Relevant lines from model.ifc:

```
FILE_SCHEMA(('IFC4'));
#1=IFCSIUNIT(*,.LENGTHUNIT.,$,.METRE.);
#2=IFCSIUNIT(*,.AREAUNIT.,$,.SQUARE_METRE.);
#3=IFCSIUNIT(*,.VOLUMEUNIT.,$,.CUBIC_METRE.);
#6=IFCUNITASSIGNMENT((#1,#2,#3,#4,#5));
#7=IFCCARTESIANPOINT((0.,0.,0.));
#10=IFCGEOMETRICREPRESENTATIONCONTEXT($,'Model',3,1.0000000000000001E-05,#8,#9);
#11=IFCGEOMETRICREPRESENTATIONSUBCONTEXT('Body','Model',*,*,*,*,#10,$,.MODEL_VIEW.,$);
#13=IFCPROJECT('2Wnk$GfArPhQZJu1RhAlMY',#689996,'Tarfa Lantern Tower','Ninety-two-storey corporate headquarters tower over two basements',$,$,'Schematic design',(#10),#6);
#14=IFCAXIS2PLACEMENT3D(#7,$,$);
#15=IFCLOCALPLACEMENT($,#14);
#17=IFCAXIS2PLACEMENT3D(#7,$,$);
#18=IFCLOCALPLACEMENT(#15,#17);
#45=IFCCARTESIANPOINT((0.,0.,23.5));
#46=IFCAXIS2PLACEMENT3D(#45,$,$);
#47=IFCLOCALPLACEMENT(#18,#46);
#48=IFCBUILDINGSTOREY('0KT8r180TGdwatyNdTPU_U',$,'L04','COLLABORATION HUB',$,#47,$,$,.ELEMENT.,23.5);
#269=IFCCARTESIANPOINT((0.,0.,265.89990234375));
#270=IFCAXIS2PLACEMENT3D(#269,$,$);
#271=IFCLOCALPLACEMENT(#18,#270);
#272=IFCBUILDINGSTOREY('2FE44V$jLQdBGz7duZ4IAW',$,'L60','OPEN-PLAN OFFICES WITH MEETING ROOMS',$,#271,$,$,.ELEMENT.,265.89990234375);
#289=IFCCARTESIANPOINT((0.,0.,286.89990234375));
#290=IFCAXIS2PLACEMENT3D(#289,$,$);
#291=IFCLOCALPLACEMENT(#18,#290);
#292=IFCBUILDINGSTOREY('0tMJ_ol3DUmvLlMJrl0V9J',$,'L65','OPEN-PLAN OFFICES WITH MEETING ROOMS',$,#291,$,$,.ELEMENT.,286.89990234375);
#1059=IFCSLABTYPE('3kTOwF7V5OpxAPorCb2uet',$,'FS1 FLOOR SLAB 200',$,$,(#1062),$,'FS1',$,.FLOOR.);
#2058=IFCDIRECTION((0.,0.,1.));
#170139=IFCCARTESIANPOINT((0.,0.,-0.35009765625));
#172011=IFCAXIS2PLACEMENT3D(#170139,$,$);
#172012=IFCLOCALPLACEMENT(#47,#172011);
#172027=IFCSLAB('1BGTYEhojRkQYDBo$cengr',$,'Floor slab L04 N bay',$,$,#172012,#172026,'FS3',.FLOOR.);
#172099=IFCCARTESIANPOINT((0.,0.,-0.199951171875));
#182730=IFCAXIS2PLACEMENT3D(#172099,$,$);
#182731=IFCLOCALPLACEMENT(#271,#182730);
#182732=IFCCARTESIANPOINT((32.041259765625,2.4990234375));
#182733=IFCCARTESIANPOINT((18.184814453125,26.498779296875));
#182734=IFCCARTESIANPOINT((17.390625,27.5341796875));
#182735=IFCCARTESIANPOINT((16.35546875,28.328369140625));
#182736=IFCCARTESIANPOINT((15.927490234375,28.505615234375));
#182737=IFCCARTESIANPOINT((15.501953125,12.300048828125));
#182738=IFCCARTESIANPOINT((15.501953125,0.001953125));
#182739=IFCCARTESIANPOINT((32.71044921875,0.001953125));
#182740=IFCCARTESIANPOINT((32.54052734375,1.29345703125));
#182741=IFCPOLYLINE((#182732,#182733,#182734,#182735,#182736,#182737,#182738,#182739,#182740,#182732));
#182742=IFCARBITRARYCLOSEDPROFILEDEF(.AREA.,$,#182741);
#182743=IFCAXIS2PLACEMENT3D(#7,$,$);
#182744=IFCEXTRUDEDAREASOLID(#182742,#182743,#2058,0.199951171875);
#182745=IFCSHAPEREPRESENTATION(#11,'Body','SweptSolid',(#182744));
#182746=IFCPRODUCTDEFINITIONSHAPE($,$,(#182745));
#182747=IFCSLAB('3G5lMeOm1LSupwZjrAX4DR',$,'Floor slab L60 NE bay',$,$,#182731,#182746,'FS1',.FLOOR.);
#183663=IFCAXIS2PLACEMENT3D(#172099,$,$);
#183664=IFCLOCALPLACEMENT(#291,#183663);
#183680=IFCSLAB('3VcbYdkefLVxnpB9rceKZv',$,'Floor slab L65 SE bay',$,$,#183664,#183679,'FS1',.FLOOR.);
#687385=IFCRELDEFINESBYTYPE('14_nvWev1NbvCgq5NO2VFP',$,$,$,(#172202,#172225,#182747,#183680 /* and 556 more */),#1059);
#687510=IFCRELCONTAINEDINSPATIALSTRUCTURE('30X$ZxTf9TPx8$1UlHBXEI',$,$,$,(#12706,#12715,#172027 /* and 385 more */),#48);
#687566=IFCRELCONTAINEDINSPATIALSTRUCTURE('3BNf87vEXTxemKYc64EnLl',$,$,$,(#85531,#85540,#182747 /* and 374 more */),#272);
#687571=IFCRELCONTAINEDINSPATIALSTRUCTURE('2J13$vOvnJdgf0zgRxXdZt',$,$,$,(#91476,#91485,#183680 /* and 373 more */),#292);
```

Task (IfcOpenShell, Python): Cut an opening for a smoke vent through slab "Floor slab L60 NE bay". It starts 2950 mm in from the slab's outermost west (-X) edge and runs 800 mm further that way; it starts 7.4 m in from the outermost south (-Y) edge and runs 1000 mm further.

```python
import numpy as np
import ifcopenshell
import ifcopenshell.api.feature
import ifcopenshell.api.geometry
import ifcopenshell.api.root
import ifcopenshell.geom
import ifcopenshell.util.placement
import ifcopenshell.util.representation
import ifcopenshell.util.shape
import ifcopenshell.util.unit

model = ifcopenshell.open("model.ifc")
unit_scale = ifcopenshell.util.unit.calculate_unit_scale(model)
settings = ifcopenshell.geom.settings()


def volume(element):
    """Net volume in cubic metres, openings subtracted."""
    shape = ifcopenshell.geom.create_shape(settings, element)
    return ifcopenshell.util.shape.get_volume(shape.geometry)


slab = model.by_guid("3G5lMeOm1LSupwZjrAX4DR")
before = volume(slab)

# Extent in the slab's own axes, in metres. The edges named are its -X and -Y sides.
slab_shape = ifcopenshell.geom.create_shape(settings, slab)
vertices = ifcopenshell.util.shape.get_vertices(slab_shape.geometry)
x_min, y_min, bottom = vertices.min(axis=0)
top = vertices[:, 2].max()

opening = ifcopenshell.api.root.create_entity(model, ifc_class="IfcOpeningElement", name="Smoke vent opening", predefined_type="OPENING")
context = ifcopenshell.util.representation.get_context(model, "Model", "Body", "MODEL_VIEW")
width, depth = 0.8, 1
outline = [(0.0, 0.0), (width, 0.0), (width, depth), (0.0, depth), (0.0, 0.0)]
# Overshoot both faces by 50 mm so the cut is clean.
shape = ifcopenshell.api.geometry.add_slab_representation(
    model, context=context, depth=top - bottom + 0.1, polyline=outline
)
ifcopenshell.api.geometry.assign_representation(model, product=opening, representation=shape)

matrix = ifcopenshell.util.placement.get_local_placement(slab.ObjectPlacement)
matrix[:, 3] = matrix @ np.append(np.array([x_min + 2.95, y_min + 7.4, bottom - 0.05]) / unit_scale, 1.0)
ifcopenshell.api.geometry.edit_object_placement(model, product=opening, matrix=matrix, is_si=False)
ifcopenshell.api.feature.add_feature(model, feature=opening, element=slab)

after = volume(slab)

print(f"slab volume {before:.3f} -> {after:.3f} m3")

model.write("model_rev.ifc")
```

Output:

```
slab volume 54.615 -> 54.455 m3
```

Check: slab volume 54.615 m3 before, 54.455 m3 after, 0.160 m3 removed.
